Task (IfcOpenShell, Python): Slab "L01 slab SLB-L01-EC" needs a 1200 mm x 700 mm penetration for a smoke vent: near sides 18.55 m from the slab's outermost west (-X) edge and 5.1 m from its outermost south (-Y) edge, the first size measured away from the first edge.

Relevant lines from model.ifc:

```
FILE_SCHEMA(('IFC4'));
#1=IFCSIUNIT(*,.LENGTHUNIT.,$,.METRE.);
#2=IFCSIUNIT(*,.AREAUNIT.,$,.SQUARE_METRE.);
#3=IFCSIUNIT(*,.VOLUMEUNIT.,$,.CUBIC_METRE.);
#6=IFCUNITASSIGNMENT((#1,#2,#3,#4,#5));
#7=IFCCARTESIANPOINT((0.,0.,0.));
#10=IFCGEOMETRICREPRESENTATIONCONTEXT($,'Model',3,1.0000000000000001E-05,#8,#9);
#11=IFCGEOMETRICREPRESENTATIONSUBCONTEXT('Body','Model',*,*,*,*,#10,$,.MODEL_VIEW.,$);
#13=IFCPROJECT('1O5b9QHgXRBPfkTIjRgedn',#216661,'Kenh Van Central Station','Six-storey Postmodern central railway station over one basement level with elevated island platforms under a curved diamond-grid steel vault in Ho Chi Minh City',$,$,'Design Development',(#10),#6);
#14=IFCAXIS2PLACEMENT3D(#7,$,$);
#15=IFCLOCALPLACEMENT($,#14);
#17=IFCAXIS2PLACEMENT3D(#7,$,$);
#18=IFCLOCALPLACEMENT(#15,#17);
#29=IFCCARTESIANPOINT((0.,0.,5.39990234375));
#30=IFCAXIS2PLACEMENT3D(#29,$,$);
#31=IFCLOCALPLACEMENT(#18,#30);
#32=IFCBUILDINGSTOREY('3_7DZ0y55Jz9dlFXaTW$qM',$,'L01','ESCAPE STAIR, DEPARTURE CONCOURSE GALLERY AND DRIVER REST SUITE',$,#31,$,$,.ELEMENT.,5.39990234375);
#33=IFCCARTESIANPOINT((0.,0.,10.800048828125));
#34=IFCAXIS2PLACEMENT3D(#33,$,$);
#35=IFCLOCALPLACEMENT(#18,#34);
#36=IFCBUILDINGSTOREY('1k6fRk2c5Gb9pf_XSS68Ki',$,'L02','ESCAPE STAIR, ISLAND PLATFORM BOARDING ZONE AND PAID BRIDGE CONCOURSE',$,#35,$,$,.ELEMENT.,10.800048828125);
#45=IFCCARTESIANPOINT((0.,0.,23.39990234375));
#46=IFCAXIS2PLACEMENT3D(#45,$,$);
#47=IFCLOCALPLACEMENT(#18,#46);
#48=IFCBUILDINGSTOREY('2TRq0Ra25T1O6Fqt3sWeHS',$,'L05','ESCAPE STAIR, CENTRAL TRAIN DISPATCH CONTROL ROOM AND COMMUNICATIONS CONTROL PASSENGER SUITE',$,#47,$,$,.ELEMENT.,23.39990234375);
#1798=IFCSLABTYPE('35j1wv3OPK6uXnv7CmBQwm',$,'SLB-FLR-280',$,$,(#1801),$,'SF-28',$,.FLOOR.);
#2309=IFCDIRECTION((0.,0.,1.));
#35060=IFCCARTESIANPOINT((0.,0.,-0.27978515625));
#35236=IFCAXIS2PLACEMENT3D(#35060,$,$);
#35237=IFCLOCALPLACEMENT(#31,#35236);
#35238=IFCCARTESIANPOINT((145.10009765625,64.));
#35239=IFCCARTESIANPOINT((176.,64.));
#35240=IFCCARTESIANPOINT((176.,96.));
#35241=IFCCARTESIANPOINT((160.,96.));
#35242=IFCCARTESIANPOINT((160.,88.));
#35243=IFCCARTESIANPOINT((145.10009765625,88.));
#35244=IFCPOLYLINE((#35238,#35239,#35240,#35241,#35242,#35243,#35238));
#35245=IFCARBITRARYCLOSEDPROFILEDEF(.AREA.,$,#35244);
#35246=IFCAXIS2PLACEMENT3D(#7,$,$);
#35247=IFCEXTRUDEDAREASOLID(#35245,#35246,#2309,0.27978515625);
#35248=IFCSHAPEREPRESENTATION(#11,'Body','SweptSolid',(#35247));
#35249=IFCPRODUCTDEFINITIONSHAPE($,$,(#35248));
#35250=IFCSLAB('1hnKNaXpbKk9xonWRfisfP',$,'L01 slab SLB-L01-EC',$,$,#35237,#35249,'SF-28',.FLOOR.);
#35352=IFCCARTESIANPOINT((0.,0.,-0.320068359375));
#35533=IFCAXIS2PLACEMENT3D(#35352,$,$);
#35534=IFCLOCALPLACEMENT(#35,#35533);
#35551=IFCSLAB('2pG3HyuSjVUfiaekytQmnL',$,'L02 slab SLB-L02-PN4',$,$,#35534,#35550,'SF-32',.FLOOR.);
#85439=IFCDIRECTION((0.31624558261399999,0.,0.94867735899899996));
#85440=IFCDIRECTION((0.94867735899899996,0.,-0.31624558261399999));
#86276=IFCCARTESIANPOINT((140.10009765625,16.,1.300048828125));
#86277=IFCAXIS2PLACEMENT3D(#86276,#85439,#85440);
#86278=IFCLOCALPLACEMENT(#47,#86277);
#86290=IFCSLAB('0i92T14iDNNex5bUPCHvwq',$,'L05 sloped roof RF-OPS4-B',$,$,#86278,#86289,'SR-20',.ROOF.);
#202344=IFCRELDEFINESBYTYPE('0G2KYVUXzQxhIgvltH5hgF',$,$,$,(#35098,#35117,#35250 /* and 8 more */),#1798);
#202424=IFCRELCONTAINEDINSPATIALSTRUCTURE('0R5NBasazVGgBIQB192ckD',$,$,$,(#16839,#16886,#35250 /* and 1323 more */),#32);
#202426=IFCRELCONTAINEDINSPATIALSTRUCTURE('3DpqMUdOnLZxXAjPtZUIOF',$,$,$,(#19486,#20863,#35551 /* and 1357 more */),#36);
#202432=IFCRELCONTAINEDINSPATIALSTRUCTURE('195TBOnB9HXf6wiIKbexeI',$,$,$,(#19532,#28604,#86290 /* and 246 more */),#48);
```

```python
import numpy as np
import ifcopenshell
import ifcopenshell.api.feature
import ifcopenshell.api.geometry
import ifcopenshell.api.root
import ifcopenshell.geom
import ifcopenshell.util.placement
import ifcopenshell.util.representation
import ifcopenshell.util.shape
import ifcopenshell.util.unit

model = ifcopenshell.open("model.ifc")
unit_scale = ifcopenshell.util.unit.calculate_unit_scale(model)
settings = ifcopenshell.geom.settings()


def volume(element):
    """Net volume in cubic metres, openings subtracted."""
    shape = ifcopenshell.geom.create_shape(settings, element)
    return ifcopenshell.util.shape.get_volume(shape.geometry)


slab = model.by_guid("1hnKNaXpbKk9xonWRfisfP")
before = volume(slab)

# Extent in the slab's own axes, in metres. The edges named are its -X and -Y sides.
slab_shape = ifcopenshell.geom.create_shape(settings, slab)
vertices = ifcopenshell.util.shape.get_vertices(slab_shape.geometry)
x_min, y_min, bottom = vertices.min(axis=0)
top = vertices[:, 2].max()

opening = ifcopenshell.api.root.create_entity(model, ifc_class="IfcOpeningElement", name="Smoke vent opening", predefined_type="OPENING")
context = ifcopenshell.util.representation.get_context(model, "Model", "Body", "MODEL_VIEW")
width, depth = 1.2, 0.7
outline = [(0.0, 0.0), (width, 0.0), (width, depth), (0.0, depth), (0.0, 0.0)]
# Overshoot both faces by 50 mm so the cut is clean.
shape = ifcopenshell.api.geometry.add_slab_representation(
    model, context=context, depth=top - bottom + 0.1, polyline=outline
)
ifcopenshell.api.geometry.assign_representation(model, product=opening, representation=shape)

matrix = ifcopenshell.util.placement.get_local_placement(slab.ObjectPlacement)
matrix[:, 3] = matrix @ np.append(np.array([x_min + 18.55, y_min + 5.1, bottom - 0.05]) / unit_scale, 1.0)
ifcopenshell.api.geometry.edit_object_placement(model, product=opening, matrix=matrix, is_si=False)
ifcopenshell.api.feature.add_feature(model, feature=opening, element=slab)

after = volume(slab)

print(f"slab volume {before:.3f} -> {after:.3f} m3")

model.write("model-out.ifc")
```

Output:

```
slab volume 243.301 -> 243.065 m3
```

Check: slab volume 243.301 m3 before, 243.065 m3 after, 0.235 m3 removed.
